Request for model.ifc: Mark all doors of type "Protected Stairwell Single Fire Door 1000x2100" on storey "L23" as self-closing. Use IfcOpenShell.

First a look at what the model holds.

```python
import ifcopenshell
import ifcopenshell.util.element

model = ifcopenshell.open("model.ifc")
print(model.schema)
storey = next(s for s in model.by_type("IfcBuildingStorey") if s.Name == "L23")
doors = [e for e in ifcopenshell.util.element.get_decomposition(storey) if e.is_a("IfcDoor")]
seen = {}
for e in doors:
    element_type = ifcopenshell.util.element.get_type(e)
    key = (element_type.Name if element_type != e and element_type else None, ifcopenshell.util.element.get_pset(e, "Pset_DoorCommon", "SelfClosing"))
    seen[key] = seen.get(key, 0) + 1
for (name, value), count in sorted(seen.items(), key=str):
    print(count, "x", name, "|", value)
```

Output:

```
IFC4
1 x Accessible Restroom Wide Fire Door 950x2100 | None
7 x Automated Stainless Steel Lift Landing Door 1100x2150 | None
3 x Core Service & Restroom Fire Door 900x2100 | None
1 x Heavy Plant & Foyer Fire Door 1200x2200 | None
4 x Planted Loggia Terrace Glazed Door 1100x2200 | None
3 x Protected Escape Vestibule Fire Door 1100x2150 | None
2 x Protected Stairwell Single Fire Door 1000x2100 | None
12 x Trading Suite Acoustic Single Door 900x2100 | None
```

```python
import ifcopenshell
import ifcopenshell.api.pset
import ifcopenshell.util.element

model = ifcopenshell.open("model.ifc")

storey = next(s for s in model.by_type("IfcBuildingStorey") if s.Name == "L23")
doors = [e for e in ifcopenshell.util.element.get_decomposition(storey) if e.is_a("IfcDoor")]

count = 0
for e in doors:
    element_type = ifcopenshell.util.element.get_type(e)
    if element_type in (None, e) or element_type.Name != "Protected Stairwell Single Fire Door 1000x2100":
        continue
    # add_pset returns the element's existing set when there is one.
    pset = ifcopenshell.api.pset.add_pset(model, product=e, name="Pset_DoorCommon")
    ifcopenshell.api.pset.edit_pset(model, pset=pset, properties={"SelfClosing": True})
    count += 1

print(count, "doors updated")

model.write("model_edited.ifc")
```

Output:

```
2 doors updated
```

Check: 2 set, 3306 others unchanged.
